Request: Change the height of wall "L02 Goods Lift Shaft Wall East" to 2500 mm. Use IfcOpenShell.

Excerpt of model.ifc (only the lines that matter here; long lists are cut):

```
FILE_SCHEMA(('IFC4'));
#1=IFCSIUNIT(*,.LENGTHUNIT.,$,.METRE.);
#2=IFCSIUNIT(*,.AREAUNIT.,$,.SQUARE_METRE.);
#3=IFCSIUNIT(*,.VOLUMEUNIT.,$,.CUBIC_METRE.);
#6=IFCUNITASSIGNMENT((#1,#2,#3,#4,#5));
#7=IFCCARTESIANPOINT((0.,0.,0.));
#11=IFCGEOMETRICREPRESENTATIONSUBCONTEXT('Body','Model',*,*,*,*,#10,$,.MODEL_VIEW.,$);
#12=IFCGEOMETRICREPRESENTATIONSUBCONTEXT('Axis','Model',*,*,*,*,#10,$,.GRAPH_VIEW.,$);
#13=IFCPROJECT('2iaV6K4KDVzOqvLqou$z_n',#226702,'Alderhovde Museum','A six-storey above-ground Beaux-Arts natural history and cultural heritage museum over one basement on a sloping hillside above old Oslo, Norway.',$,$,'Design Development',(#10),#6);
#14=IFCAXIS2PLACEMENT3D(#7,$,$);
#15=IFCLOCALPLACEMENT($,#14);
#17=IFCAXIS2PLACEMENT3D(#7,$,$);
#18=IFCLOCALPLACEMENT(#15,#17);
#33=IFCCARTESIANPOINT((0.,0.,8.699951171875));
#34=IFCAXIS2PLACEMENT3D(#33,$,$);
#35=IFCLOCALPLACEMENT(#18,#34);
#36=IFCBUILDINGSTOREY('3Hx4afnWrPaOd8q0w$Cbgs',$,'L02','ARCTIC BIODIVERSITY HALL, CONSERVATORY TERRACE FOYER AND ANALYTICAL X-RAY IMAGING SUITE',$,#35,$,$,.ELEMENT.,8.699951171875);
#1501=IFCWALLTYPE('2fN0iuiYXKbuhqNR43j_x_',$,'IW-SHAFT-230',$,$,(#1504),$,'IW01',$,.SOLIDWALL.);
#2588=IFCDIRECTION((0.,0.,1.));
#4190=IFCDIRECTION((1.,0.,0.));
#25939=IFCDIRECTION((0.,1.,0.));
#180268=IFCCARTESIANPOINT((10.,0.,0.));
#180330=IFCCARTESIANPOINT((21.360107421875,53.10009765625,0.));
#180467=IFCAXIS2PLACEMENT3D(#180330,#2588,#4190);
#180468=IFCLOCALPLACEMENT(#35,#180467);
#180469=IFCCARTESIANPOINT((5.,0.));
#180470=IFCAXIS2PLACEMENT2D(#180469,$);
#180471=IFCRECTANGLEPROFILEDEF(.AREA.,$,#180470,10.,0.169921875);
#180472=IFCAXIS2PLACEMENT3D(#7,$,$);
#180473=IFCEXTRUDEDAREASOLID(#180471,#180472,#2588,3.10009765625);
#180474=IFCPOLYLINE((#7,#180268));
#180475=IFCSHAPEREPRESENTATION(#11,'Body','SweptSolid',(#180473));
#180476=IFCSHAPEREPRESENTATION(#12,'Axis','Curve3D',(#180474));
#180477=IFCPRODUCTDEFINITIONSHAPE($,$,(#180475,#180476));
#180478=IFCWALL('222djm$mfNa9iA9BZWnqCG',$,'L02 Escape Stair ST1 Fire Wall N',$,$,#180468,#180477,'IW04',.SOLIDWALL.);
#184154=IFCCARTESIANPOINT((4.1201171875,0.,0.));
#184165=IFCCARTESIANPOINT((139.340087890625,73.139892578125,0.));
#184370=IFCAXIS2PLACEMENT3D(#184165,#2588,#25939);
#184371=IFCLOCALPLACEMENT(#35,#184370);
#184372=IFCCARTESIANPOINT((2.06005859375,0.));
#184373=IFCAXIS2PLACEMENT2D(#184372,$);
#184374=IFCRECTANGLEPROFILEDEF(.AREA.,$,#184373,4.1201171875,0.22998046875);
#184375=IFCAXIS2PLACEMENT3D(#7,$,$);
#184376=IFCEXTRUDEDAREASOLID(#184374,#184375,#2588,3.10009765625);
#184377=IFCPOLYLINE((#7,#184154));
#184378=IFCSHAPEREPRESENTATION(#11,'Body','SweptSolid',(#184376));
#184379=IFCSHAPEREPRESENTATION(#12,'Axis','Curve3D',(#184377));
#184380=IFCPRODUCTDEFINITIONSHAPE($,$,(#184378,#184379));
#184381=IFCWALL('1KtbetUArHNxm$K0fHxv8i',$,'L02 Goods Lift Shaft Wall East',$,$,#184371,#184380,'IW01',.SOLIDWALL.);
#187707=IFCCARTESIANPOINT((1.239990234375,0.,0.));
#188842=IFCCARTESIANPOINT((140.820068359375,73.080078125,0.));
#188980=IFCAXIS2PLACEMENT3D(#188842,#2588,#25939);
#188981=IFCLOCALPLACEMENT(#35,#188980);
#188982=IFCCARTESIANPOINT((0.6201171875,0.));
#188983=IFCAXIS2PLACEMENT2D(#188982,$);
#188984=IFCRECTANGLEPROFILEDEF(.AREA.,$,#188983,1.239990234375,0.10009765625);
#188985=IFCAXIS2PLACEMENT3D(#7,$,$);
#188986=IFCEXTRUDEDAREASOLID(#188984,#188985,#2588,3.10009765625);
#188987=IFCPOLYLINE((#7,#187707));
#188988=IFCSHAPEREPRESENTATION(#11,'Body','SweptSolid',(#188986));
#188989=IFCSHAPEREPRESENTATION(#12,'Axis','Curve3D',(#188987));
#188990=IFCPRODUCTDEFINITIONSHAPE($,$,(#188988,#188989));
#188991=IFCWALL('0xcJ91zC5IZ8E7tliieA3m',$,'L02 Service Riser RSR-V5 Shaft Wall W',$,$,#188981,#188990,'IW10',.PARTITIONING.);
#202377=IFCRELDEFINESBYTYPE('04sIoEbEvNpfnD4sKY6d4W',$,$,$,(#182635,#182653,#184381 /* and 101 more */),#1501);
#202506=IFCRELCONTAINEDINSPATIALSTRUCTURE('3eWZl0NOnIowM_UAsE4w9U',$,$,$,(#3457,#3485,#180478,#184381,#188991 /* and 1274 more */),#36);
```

```python
import ifcopenshell
import ifcopenshell.geom
import ifcopenshell.util.representation
import ifcopenshell.util.shape
import ifcopenshell.util.unit

model = ifcopenshell.open("model.ifc")
unit_scale = ifcopenshell.util.unit.calculate_unit_scale(model)
settings = ifcopenshell.geom.settings()


def volume(element):
    """Net volume in cubic metres, openings subtracted."""
    shape = ifcopenshell.geom.create_shape(settings, element)
    return ifcopenshell.util.shape.get_volume(shape.geometry)


wall = model.by_guid("1KtbetUArHNxm$K0fHxv8i")
before = volume(wall)

body = ifcopenshell.util.representation.get_representation(wall, "Model", "Body")
solid = body.Items[0]
old_height = solid.Depth
solid.Depth = 2.5 / unit_scale
after = volume(wall)

print(f"height {old_height:g} -> {solid.Depth:g}, volume {before:.3f} -> {after:.3f} m3")

model.write("model_updated.ifc")
```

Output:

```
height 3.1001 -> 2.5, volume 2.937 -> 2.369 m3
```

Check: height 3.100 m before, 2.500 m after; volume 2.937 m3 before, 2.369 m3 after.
